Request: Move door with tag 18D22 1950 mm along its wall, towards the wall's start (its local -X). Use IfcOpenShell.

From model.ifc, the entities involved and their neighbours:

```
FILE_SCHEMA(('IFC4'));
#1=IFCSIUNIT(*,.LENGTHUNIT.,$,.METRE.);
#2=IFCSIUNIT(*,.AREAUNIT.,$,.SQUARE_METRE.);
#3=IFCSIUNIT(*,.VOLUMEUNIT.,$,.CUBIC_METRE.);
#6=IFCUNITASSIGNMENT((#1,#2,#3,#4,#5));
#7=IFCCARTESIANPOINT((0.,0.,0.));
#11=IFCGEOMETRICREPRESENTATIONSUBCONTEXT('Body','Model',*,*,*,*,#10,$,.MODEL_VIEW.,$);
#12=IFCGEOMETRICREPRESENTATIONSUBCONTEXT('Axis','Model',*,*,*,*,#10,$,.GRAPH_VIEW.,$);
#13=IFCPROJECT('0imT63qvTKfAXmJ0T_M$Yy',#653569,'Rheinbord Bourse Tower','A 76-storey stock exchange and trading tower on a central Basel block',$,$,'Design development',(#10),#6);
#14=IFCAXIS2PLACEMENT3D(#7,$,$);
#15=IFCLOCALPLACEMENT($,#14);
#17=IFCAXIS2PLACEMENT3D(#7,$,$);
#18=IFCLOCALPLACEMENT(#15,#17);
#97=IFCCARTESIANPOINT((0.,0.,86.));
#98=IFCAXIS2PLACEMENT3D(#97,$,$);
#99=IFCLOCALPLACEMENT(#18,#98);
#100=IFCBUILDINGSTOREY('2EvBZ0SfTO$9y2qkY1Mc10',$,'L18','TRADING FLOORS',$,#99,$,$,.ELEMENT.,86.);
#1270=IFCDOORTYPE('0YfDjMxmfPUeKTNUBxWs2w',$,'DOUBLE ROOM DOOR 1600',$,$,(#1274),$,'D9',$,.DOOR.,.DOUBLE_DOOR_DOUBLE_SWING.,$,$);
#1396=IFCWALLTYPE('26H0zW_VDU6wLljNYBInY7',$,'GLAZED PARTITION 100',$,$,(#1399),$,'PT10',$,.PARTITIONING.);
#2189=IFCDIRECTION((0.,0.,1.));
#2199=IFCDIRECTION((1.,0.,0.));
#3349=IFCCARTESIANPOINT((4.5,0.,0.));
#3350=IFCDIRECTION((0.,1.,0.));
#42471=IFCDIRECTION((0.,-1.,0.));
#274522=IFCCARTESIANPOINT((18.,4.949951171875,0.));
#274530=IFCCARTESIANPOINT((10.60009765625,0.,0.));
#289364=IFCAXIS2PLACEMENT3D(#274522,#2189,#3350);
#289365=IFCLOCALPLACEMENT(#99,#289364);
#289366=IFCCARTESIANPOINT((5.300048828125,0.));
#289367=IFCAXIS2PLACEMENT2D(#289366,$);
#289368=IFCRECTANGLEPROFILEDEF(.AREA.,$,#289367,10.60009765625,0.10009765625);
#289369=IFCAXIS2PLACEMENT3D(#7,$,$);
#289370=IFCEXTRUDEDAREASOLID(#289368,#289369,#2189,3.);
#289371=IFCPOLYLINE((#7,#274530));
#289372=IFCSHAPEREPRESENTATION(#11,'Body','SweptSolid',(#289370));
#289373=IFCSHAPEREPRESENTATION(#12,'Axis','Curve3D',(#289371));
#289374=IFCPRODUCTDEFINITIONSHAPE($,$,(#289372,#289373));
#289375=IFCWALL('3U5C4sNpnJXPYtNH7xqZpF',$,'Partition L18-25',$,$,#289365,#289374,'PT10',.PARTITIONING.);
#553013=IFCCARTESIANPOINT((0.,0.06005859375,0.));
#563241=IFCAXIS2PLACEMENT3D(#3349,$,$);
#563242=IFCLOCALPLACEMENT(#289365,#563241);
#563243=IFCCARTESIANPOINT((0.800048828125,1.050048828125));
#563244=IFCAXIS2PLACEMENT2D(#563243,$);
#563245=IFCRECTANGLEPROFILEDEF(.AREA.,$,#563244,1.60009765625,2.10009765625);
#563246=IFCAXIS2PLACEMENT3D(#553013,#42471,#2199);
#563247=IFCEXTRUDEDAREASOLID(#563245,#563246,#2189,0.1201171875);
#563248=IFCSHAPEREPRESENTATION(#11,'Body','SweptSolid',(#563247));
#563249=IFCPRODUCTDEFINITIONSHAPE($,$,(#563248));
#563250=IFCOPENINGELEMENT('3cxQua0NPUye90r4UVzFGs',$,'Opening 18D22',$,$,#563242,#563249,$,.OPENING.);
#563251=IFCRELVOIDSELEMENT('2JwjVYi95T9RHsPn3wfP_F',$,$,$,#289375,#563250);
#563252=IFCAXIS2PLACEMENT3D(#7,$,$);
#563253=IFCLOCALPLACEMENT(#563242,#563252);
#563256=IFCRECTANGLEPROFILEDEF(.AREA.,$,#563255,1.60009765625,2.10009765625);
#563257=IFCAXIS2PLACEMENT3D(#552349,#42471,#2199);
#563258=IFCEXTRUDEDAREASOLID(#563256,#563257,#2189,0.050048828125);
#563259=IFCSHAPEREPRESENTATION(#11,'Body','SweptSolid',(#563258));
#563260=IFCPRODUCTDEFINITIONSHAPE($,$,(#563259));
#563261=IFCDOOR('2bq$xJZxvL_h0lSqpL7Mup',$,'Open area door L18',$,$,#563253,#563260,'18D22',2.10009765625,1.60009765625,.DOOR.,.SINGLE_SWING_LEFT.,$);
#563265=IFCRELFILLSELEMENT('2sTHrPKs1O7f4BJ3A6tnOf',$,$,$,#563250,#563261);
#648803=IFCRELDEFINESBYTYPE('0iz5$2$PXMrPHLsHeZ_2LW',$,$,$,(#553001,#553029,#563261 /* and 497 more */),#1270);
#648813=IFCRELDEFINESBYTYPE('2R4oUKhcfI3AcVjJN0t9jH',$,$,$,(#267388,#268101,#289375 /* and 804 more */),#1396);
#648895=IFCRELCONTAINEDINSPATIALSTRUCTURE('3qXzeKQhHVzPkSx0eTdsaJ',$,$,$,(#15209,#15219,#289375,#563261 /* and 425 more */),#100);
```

```python
import ifcopenshell
import ifcopenshell.api.geometry
import ifcopenshell.util.placement
import ifcopenshell.util.unit

model = ifcopenshell.open("model.ifc")
unit_scale = ifcopenshell.util.unit.calculate_unit_scale(model)

door = model.by_guid("2bq$xJZxvL_h0lSqpL7Mup")
opening = door.FillsVoids[0].RelatingOpeningElement
wall = opening.VoidsElements[0].RelatingBuildingElement

wall_matrix = ifcopenshell.util.placement.get_local_placement(wall.ObjectPlacement)
shift = wall_matrix[:3, 0] * -1.95 / unit_scale
before = ifcopenshell.util.placement.get_local_placement(door.ObjectPlacement)[:3, 3].copy()

# The door is placed relative to its opening, so it follows when the opening moves.
matrix = ifcopenshell.util.placement.get_local_placement(opening.ObjectPlacement)
matrix[:3, 3] += shift
ifcopenshell.api.geometry.edit_object_placement(
    model, product=opening, matrix=matrix, is_si=False, should_transform_children=True
)

after = ifcopenshell.util.placement.get_local_placement(door.ObjectPlacement)[:3, 3]
print("door moved by", (after - before).round(3) + 0.0)

model.write("model_v2.ifc")
```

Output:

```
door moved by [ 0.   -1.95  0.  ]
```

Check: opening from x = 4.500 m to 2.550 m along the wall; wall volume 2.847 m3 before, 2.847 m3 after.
